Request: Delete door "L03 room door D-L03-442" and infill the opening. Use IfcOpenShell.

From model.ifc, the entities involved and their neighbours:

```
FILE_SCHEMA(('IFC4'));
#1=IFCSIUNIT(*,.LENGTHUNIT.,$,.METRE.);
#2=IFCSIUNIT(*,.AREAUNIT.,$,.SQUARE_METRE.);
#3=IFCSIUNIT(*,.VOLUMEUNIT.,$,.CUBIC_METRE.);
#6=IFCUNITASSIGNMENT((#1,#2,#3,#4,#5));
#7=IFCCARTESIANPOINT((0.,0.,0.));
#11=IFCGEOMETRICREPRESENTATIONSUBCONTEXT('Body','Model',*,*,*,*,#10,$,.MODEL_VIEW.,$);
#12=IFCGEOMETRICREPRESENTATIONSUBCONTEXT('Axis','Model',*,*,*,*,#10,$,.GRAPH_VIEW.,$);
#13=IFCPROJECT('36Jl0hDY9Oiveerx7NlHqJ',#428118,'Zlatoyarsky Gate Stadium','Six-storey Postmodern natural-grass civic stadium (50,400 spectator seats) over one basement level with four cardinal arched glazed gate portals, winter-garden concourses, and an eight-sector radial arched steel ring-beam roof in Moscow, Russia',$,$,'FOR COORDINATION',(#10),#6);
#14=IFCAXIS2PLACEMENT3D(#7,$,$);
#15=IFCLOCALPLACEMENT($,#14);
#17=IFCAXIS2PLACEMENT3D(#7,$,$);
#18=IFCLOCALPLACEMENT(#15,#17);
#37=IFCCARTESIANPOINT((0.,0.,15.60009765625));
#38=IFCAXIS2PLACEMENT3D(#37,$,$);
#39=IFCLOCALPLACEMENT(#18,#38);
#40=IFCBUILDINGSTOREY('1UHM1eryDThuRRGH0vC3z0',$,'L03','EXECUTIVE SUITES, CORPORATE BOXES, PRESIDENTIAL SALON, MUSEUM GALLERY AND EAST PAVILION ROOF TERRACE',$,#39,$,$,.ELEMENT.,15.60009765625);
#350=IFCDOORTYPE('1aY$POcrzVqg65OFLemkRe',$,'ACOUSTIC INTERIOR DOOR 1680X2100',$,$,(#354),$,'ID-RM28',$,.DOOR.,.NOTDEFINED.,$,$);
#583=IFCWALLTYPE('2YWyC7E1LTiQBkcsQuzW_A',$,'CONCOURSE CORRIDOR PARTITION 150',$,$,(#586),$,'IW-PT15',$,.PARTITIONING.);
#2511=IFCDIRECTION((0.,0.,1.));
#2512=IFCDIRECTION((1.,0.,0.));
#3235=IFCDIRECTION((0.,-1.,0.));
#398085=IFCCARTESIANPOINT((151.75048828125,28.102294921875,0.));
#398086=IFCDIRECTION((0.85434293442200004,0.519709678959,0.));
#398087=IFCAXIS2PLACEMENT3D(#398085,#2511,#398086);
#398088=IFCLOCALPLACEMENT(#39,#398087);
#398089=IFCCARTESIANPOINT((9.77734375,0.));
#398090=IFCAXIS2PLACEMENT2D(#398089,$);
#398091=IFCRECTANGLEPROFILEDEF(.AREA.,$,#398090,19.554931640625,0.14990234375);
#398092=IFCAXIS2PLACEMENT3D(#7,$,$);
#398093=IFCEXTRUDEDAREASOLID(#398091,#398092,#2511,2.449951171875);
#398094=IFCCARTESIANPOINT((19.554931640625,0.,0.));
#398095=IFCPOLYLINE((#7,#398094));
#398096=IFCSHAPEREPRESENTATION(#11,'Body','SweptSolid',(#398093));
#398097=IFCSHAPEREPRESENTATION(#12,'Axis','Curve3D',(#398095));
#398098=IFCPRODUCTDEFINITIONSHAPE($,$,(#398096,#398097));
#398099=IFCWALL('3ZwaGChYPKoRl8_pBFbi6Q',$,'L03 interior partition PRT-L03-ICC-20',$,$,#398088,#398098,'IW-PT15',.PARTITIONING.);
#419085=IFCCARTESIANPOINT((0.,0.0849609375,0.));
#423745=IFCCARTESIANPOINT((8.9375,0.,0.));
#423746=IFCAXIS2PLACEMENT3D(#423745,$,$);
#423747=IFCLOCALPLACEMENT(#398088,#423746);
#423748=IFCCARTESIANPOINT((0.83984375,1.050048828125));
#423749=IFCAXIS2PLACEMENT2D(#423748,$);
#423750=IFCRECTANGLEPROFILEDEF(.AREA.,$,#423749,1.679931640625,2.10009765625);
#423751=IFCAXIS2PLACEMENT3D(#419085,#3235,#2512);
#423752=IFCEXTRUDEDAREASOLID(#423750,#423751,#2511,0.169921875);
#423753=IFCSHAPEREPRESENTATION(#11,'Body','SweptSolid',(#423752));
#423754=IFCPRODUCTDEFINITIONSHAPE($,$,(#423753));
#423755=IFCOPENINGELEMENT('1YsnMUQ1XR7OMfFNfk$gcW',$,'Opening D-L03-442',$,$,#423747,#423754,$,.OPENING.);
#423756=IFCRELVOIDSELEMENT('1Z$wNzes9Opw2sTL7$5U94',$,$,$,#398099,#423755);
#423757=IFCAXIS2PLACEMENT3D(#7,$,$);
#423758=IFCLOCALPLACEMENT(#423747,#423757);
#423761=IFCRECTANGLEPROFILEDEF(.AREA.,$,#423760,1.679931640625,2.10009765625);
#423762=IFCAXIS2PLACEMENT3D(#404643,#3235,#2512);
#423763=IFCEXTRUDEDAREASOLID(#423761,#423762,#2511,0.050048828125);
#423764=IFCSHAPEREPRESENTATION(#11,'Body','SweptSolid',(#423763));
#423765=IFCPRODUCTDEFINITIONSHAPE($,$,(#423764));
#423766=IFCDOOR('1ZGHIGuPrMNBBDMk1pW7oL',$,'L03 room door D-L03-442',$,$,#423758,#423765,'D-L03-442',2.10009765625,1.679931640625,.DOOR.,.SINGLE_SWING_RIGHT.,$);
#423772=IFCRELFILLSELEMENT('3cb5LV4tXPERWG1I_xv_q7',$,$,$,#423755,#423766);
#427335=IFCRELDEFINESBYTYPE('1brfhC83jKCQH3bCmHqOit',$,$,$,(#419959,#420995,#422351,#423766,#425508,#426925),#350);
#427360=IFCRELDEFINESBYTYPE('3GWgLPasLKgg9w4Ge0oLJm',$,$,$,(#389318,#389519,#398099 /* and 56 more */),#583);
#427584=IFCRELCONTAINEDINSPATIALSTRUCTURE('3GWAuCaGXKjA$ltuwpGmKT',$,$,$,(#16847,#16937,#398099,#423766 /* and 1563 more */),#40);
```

```python
import ifcopenshell
import ifcopenshell.api.feature
import ifcopenshell.api.root
import ifcopenshell.geom
import ifcopenshell.util.shape

model = ifcopenshell.open("model.ifc")
settings = ifcopenshell.geom.settings()


def volume(element):
    """Net volume in cubic metres, openings subtracted."""
    shape = ifcopenshell.geom.create_shape(settings, element)
    return ifcopenshell.util.shape.get_volume(shape.geometry)


door = model.by_guid("1ZGHIGuPrMNBBDMk1pW7oL")
opening = door.FillsVoids[0].RelatingOpeningElement
wall = opening.VoidsElements[0].RelatingBuildingElement
before = volume(wall)

ifcopenshell.api.root.remove_product(model, product=door)
ifcopenshell.api.feature.remove_feature(model, feature=opening)

after = volume(wall)

print(f"wall volume {before:.3f} -> {after:.3f} m3")

model.write("model_edited.ifc")
```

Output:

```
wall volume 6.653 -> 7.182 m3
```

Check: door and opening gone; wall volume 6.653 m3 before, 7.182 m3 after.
